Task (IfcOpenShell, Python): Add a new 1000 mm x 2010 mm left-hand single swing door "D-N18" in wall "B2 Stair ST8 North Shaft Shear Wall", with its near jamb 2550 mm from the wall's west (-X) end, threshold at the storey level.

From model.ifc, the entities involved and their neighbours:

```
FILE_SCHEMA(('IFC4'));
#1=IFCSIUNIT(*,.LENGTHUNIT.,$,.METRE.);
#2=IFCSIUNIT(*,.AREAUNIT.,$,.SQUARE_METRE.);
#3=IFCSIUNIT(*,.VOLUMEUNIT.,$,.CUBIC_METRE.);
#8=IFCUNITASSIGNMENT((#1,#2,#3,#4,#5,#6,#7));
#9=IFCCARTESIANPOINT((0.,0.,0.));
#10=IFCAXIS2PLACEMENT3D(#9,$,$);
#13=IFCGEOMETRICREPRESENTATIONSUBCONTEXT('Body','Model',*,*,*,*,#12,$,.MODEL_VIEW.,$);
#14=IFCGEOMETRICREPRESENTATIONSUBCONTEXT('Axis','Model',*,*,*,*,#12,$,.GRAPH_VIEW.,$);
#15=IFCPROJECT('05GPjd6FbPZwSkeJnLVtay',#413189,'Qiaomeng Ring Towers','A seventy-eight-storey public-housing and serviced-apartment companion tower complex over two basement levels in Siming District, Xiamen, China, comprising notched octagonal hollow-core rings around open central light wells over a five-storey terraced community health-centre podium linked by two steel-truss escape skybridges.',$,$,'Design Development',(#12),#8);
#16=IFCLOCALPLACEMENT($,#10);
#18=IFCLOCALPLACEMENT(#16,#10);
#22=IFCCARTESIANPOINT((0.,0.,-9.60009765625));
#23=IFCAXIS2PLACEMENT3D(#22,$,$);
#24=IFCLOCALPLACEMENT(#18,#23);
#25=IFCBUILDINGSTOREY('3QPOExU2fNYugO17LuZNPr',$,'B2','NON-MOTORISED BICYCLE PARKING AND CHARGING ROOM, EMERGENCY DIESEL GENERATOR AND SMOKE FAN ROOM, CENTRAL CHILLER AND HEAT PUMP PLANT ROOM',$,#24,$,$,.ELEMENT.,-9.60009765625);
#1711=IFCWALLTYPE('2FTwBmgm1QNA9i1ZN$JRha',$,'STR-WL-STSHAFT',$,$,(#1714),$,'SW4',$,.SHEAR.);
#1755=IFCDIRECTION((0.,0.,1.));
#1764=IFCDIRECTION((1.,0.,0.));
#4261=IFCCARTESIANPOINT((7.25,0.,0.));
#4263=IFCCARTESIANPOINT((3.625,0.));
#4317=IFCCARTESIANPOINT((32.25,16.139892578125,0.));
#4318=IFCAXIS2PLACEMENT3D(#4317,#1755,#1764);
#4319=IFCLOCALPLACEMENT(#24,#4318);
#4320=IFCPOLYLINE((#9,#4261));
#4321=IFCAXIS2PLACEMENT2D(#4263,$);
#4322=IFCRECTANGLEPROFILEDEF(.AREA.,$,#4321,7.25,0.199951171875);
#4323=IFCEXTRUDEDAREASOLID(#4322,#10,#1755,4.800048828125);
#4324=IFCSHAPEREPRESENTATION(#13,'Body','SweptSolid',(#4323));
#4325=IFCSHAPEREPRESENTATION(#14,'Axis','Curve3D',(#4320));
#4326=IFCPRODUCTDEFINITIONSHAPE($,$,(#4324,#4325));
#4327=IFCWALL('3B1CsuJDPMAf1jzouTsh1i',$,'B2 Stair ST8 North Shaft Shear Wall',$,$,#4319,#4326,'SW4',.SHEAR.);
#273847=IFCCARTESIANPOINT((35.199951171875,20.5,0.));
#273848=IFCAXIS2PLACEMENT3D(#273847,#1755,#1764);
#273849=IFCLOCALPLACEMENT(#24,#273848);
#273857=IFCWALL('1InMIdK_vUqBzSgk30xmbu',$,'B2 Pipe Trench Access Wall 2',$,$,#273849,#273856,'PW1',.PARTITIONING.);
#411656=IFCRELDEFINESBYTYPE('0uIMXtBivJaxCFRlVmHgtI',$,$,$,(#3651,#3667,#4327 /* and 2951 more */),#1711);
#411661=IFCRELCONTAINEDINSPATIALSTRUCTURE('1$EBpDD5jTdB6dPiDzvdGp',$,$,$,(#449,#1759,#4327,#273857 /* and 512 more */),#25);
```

```python
import numpy as np
import ifcopenshell
import ifcopenshell.api.feature
import ifcopenshell.api.geometry
import ifcopenshell.api.root
import ifcopenshell.api.spatial
import ifcopenshell.geom
import ifcopenshell.util.element
import ifcopenshell.util.placement
import ifcopenshell.util.representation
import ifcopenshell.util.shape
import ifcopenshell.util.unit

model = ifcopenshell.open("model.ifc")
unit_scale = ifcopenshell.util.unit.calculate_unit_scale(model)
settings = ifcopenshell.geom.settings()


def volume(element):
    """Net volume in cubic metres, openings subtracted."""
    shape = ifcopenshell.geom.create_shape(settings, element)
    return ifcopenshell.util.shape.get_volume(shape.geometry)


wall = model.by_guid("3B1CsuJDPMAf1jzouTsh1i")
storey = ifcopenshell.util.element.get_container(wall, ifc_class="IfcBuildingStorey")
context = ifcopenshell.util.representation.get_context(model, "Model", "Body", "MODEL_VIEW")
before = volume(wall)

width, height, from_end, sill = 1, 2.01, 2.55, 0.0  # metres

# The wall runs along its own X axis, and the end named is its -X end.
wall_shape = ifcopenshell.geom.create_shape(settings, wall)
x, y, z = ifcopenshell.util.shape.get_vertices(wall_shape.geometry).T
start = x.min() + from_end
face, thickness = float(y.min()), float(y.max() - y.min())
wall_matrix = ifcopenshell.util.placement.get_local_placement(wall.ObjectPlacement)
level = ifcopenshell.util.placement.get_local_placement(storey.ObjectPlacement)[2, 3]


def in_wall(x, y):
    """Placement at x, y metres in the wall's axes, at sill height."""
    matrix = wall_matrix.copy()
    matrix[:, 3] = wall_matrix @ np.array([x / unit_scale, y / unit_scale, 0.0, 1.0])
    matrix[2, 3] = level + sill / unit_scale
    return matrix


# Opening: a box that overshoots both wall faces by 50 mm.
opening = ifcopenshell.api.root.create_entity(model, ifc_class="IfcOpeningElement", predefined_type="OPENING")
box = ifcopenshell.api.geometry.add_wall_representation(
    model, context=context, length=width, height=height, thickness=thickness + 0.1
)
ifcopenshell.api.geometry.assign_representation(model, product=opening, representation=box)
ifcopenshell.api.geometry.edit_object_placement(model, product=opening, matrix=in_wall(start, face - 0.05), is_si=False)
ifcopenshell.api.feature.add_feature(model, feature=opening, element=wall)

door = ifcopenshell.api.root.create_entity(model, ifc_class="IfcDoor", name="D-N18", predefined_type="DOOR")
door.OverallWidth, door.OverallHeight = width / unit_scale, height / unit_scale
door.OperationType = "SINGLE_SWING_LEFT"
body = ifcopenshell.api.geometry.add_door_representation(
    model,
    context=context,
    overall_width=door.OverallWidth,
    overall_height=door.OverallHeight,
    operation_type="SINGLE_SWING_LEFT",
    lining_properties={"LiningDepth": thickness / unit_scale, "ThresholdDepth": thickness / unit_scale},
)
ifcopenshell.api.geometry.assign_representation(model, product=door, representation=body)
ifcopenshell.api.spatial.assign_container(model, products=[door], relating_structure=storey)
ifcopenshell.api.feature.add_filling(model, opening=opening, element=door)

# The lining spans the wall, so the door starts at the wall face.
ifcopenshell.api.geometry.edit_object_placement(model, product=door, matrix=in_wall(start, face), is_si=False)

after = volume(wall)

print(f"wall volume {before:.3f} -> {after:.3f} m3")

model.write("model_rev.ifc")
```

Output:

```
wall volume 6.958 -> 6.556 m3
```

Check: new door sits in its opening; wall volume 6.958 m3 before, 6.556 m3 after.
